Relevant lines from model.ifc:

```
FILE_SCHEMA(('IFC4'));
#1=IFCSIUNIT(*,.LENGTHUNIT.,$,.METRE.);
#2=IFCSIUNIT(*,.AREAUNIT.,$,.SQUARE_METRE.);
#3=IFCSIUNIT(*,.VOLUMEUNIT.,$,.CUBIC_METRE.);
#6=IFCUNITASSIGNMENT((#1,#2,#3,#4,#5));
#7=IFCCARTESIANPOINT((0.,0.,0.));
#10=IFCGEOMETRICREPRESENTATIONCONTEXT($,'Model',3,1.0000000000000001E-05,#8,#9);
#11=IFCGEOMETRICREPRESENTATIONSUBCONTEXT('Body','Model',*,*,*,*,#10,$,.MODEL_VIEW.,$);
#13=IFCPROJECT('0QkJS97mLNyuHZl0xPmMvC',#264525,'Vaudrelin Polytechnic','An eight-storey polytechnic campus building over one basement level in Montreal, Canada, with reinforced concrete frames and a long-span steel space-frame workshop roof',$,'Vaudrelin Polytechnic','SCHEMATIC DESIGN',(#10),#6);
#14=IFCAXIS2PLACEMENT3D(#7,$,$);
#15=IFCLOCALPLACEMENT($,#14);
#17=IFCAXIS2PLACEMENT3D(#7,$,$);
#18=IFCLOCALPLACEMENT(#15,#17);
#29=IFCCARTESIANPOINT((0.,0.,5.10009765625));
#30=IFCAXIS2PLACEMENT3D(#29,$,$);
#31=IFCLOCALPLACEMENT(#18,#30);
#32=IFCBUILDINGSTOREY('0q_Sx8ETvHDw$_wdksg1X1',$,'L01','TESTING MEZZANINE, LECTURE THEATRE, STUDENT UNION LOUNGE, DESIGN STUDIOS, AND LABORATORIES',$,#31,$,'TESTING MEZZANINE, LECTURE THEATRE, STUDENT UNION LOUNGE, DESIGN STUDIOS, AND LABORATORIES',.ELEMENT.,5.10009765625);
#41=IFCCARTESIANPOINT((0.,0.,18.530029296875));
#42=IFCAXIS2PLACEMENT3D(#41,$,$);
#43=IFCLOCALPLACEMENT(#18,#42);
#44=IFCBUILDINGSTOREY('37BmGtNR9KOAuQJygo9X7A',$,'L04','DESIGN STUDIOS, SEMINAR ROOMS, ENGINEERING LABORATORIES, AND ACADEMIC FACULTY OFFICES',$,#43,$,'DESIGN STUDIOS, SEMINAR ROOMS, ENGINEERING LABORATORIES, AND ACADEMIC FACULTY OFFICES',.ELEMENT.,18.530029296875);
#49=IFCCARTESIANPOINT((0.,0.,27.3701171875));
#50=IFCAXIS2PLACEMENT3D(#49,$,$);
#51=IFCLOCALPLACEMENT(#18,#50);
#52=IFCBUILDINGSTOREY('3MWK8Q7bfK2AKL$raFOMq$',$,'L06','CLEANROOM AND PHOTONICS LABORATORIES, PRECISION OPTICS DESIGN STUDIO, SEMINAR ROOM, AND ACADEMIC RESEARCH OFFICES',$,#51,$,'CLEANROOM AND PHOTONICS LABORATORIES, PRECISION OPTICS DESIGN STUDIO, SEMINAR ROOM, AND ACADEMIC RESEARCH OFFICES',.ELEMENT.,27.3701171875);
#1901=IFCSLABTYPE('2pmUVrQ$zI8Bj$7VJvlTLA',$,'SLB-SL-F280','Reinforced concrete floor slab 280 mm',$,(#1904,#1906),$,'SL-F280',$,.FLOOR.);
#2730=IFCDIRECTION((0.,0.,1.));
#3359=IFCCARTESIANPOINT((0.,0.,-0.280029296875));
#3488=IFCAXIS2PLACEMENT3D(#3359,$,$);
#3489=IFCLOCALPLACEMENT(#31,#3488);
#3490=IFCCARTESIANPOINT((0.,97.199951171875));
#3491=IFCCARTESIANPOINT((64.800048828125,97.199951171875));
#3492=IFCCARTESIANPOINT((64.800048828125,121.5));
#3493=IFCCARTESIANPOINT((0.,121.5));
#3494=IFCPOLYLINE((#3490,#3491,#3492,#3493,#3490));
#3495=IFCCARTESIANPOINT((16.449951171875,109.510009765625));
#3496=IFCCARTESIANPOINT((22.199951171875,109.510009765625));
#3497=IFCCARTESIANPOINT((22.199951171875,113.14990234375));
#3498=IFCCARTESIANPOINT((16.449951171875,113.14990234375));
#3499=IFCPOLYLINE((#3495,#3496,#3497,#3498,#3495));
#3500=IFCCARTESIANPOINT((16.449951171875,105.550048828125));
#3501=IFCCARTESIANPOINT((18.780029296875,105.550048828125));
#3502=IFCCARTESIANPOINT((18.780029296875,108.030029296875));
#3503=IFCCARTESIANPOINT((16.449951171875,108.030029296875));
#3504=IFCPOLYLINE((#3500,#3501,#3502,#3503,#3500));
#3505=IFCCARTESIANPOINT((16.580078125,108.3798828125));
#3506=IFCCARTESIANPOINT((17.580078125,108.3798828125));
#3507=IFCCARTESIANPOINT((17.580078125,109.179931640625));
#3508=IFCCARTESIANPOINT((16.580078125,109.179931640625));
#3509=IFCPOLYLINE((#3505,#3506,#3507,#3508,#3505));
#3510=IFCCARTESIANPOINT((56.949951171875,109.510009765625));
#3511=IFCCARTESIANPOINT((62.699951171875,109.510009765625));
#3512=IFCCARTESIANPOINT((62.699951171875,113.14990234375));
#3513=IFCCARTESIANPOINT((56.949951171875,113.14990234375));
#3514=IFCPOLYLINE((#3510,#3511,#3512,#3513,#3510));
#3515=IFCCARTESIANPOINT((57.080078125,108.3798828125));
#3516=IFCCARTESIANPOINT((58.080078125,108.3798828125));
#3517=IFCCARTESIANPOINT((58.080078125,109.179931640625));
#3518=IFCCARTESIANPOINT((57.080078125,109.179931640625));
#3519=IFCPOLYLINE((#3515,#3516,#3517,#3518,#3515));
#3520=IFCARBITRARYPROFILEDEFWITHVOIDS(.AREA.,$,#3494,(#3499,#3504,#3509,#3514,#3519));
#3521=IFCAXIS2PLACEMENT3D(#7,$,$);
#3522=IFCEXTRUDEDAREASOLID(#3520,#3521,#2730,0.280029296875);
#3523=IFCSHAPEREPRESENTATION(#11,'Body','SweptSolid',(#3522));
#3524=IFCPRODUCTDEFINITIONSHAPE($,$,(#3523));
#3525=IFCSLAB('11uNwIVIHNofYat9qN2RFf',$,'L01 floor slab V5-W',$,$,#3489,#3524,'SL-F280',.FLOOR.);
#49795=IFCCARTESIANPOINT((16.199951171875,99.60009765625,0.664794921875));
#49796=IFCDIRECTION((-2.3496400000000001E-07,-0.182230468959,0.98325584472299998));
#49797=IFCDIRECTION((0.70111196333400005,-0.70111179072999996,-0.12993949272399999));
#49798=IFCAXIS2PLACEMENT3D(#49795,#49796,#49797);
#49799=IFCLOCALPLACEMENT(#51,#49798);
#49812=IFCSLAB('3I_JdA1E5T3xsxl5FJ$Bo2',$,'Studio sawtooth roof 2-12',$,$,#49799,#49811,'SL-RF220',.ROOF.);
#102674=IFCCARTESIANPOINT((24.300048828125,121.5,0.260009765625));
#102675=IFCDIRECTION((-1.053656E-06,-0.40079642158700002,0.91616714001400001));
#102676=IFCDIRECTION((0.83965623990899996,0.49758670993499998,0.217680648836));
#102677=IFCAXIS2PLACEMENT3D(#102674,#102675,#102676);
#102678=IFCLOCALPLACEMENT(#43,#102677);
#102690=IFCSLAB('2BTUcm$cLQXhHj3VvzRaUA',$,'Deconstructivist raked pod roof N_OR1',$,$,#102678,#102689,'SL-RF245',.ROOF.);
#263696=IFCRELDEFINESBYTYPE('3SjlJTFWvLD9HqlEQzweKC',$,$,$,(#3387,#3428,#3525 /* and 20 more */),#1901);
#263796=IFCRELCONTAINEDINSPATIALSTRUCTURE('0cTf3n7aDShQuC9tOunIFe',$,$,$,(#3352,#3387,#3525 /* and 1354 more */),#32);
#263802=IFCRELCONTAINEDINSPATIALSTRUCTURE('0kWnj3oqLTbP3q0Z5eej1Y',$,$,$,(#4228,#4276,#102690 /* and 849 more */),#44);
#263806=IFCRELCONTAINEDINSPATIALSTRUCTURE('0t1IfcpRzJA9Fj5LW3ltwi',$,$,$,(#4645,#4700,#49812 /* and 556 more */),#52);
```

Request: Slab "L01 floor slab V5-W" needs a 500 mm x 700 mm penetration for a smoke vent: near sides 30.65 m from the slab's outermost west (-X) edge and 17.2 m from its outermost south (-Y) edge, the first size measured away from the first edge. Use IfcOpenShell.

```python
import numpy as np
import ifcopenshell
import ifcopenshell.api.feature
import ifcopenshell.api.geometry
import ifcopenshell.api.root
import ifcopenshell.geom
import ifcopenshell.util.placement
import ifcopenshell.util.representation
import ifcopenshell.util.shape
import ifcopenshell.util.unit

model = ifcopenshell.open("model.ifc")
unit_scale = ifcopenshell.util.unit.calculate_unit_scale(model)
settings = ifcopenshell.geom.settings()


def volume(element):
    """Net volume in cubic metres, openings subtracted."""
    shape = ifcopenshell.geom.create_shape(settings, element)
    return ifcopenshell.util.shape.get_volume(shape.geometry)


slab = model.by_guid("11uNwIVIHNofYat9qN2RFf")
before = volume(slab)

# Extent in the slab's own axes, in metres. The edges named are its -X and -Y sides.
slab_shape = ifcopenshell.geom.create_shape(settings, slab)
vertices = ifcopenshell.util.shape.get_vertices(slab_shape.geometry)
x_min, y_min, bottom = vertices.min(axis=0)
top = vertices[:, 2].max()

opening = ifcopenshell.api.root.create_entity(model, ifc_class="IfcOpeningElement", name="Smoke vent opening", predefined_type="OPENING")
context = ifcopenshell.util.representation.get_context(model, "Model", "Body", "MODEL_VIEW")
width, depth = 0.5, 0.7
outline = [(0.0, 0.0), (width, 0.0), (width, depth), (0.0, depth), (0.0, 0.0)]
# Overshoot both faces by 50 mm so the cut is clean.
shape = ifcopenshell.api.geometry.add_slab_representation(
    model, context=context, depth=top - bottom + 0.1, polyline=outline
)
ifcopenshell.api.geometry.assign_representation(model, product=opening, representation=shape)

matrix = ifcopenshell.util.placement.get_local_placement(slab.ObjectPlacement)
matrix[:, 3] = matrix @ np.append(np.array([x_min + 30.65, y_min + 17.2, bottom - 0.05]) / unit_scale, 1.0)
ifcopenshell.api.geometry.edit_object_placement(model, product=opening, matrix=matrix, is_si=False)
ifcopenshell.api.feature.add_feature(model, feature=opening, element=slab)

after = volume(slab)

print(f"slab volume {before:.3f} -> {after:.3f} m3")

model.write("model_edited.ifc")
```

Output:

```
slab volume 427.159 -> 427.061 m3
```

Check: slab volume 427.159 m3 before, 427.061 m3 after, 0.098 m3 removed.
